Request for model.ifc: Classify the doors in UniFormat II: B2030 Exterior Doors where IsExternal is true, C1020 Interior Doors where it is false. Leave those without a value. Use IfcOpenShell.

First a look at what the model holds.

```python
import ifcopenshell
import ifcopenshell.util.element

model = ifcopenshell.open("model.ifc")
print(model.schema)
print("classifications:", [c.Name for c in model.by_type("IfcClassification")])
values = [ifcopenshell.util.element.get_pset(e, "Pset_DoorCommon", "IsExternal") for e in model.by_type("IfcDoor")]
for value in (True, False, None):
    print("IsExternal", value, values.count(value))
```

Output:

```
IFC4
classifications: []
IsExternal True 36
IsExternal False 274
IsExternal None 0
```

```python
import ifcopenshell
import ifcopenshell.api.classification
import ifcopenshell.util.element

model = ifcopenshell.open("model.ifc")

system = ifcopenshell.api.classification.add_classification(model, classification="UniFormat II")

doors = model.by_type("IfcDoor")
external = {e: ifcopenshell.util.element.get_pset(e, "Pset_DoorCommon", "IsExternal") for e in doors}
for flag, code, name in ((True, "B2030", "Exterior Doors"), (False, "C1020", "Interior Doors")):
    products = [e for e in doors if external[e] is flag]
    ifcopenshell.api.classification.add_reference(
        model, products=products, classification=system, identification=code, name=name
    )
    print(code, len(products))

model.write("model_v2.ifc")
```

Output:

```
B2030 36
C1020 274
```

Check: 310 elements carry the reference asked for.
